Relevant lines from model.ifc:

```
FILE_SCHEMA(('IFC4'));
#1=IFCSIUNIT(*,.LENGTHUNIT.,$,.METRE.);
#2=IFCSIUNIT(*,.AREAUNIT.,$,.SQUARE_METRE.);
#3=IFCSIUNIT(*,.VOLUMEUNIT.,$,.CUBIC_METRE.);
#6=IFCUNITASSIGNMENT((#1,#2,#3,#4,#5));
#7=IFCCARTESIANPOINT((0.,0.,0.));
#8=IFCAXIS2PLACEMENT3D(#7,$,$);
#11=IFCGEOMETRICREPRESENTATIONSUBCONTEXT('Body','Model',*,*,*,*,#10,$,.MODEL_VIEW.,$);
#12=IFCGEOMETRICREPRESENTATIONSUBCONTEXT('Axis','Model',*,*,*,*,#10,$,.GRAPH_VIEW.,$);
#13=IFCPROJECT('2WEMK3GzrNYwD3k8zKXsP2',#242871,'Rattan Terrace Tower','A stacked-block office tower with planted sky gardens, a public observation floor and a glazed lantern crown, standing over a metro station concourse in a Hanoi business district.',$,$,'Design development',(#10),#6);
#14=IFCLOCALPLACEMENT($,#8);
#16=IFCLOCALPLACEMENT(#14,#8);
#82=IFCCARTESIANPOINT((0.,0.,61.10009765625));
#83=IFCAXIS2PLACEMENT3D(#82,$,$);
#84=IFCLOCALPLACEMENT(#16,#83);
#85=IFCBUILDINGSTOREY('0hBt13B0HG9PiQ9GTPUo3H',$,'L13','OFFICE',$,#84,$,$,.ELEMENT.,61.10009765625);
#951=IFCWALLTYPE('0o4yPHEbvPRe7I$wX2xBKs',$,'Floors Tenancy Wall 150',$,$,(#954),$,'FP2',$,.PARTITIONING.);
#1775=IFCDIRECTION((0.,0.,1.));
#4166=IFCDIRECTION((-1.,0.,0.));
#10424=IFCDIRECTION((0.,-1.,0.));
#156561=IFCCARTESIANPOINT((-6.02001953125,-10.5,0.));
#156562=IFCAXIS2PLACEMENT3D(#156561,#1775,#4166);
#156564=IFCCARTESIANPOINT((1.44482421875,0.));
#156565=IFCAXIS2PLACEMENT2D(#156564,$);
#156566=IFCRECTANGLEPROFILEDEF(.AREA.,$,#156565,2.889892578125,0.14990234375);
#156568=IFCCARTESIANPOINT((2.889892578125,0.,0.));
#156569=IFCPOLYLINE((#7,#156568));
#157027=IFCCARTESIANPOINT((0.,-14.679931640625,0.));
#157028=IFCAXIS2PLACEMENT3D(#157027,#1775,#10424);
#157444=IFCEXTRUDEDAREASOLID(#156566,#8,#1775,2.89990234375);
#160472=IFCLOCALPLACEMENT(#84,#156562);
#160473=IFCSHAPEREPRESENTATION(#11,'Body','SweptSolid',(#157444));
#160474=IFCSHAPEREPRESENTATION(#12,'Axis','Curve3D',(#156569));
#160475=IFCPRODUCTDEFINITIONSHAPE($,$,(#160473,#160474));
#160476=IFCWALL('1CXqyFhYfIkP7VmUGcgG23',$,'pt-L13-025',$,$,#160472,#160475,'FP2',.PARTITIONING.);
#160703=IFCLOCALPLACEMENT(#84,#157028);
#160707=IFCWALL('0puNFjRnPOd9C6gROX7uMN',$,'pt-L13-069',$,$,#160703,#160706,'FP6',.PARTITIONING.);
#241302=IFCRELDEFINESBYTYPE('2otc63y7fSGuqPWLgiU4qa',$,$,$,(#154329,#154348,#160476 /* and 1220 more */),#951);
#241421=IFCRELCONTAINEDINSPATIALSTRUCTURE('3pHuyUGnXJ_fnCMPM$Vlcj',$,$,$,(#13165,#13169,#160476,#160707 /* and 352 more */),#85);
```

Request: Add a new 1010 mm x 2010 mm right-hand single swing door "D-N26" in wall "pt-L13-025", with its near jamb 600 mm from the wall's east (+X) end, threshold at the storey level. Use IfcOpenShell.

```python
import numpy as np
import ifcopenshell
import ifcopenshell.api.feature
import ifcopenshell.api.geometry
import ifcopenshell.api.root
import ifcopenshell.api.spatial
import ifcopenshell.geom
import ifcopenshell.util.element
import ifcopenshell.util.placement
import ifcopenshell.util.representation
import ifcopenshell.util.shape
import ifcopenshell.util.unit

model = ifcopenshell.open("model.ifc")
unit_scale = ifcopenshell.util.unit.calculate_unit_scale(model)
settings = ifcopenshell.geom.settings()


def volume(element):
    """Net volume in cubic metres, openings subtracted."""
    shape = ifcopenshell.geom.create_shape(settings, element)
    return ifcopenshell.util.shape.get_volume(shape.geometry)


wall = model.by_id(160476)
storey = ifcopenshell.util.element.get_container(wall, ifc_class="IfcBuildingStorey")
context = ifcopenshell.util.representation.get_context(model, "Model", "Body", "MODEL_VIEW")
before = volume(wall)

width, height, from_end, sill = 1.01, 2.01, 0.6, 0.0  # metres

# The wall runs along its own X axis, and the end named is its -X end.
wall_shape = ifcopenshell.geom.create_shape(settings, wall)
x, y, z = ifcopenshell.util.shape.get_vertices(wall_shape.geometry).T
start = x.min() + from_end
face, thickness = float(y.min()), float(y.max() - y.min())
wall_matrix = ifcopenshell.util.placement.get_local_placement(wall.ObjectPlacement)
level = ifcopenshell.util.placement.get_local_placement(storey.ObjectPlacement)[2, 3]


def in_wall(x, y):
    """Placement at x, y metres in the wall's axes, at sill height."""
    matrix = wall_matrix.copy()
    matrix[:, 3] = wall_matrix @ np.array([x / unit_scale, y / unit_scale, 0.0, 1.0])
    matrix[2, 3] = level + sill / unit_scale
    return matrix


# Opening: a box that overshoots both wall faces by 50 mm.
opening = ifcopenshell.api.root.create_entity(model, ifc_class="IfcOpeningElement", predefined_type="OPENING")
box = ifcopenshell.api.geometry.add_wall_representation(
    model, context=context, length=width, height=height, thickness=thickness + 0.1
)
ifcopenshell.api.geometry.assign_representation(model, product=opening, representation=box)
ifcopenshell.api.geometry.edit_object_placement(model, product=opening, matrix=in_wall(start, face - 0.05), is_si=False)
ifcopenshell.api.feature.add_feature(model, feature=opening, element=wall)

door = ifcopenshell.api.root.create_entity(model, ifc_class="IfcDoor", name="D-N26", predefined_type="DOOR")
door.OverallWidth, door.OverallHeight = width / unit_scale, height / unit_scale
door.OperationType = "SINGLE_SWING_RIGHT"
body = ifcopenshell.api.geometry.add_door_representation(
    model,
    context=context,
    overall_width=door.OverallWidth,
    overall_height=door.OverallHeight,
    operation_type="SINGLE_SWING_RIGHT",
    lining_properties={"LiningDepth": thickness / unit_scale, "ThresholdDepth": thickness / unit_scale},
)
ifcopenshell.api.geometry.assign_representation(model, product=door, representation=body)
ifcopenshell.api.spatial.assign_container(model, products=[door], relating_structure=storey)
ifcopenshell.api.feature.add_filling(model, opening=opening, element=door)

# The lining spans the wall, so the door starts at the wall face.
ifcopenshell.api.geometry.edit_object_placement(model, product=door, matrix=in_wall(start, face), is_si=False)

after = volume(wall)

print(f"wall volume {before:.3f} -> {after:.3f} m3")

model.write("model_v2.ifc")
```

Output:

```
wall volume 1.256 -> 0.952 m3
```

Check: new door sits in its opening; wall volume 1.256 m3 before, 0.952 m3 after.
